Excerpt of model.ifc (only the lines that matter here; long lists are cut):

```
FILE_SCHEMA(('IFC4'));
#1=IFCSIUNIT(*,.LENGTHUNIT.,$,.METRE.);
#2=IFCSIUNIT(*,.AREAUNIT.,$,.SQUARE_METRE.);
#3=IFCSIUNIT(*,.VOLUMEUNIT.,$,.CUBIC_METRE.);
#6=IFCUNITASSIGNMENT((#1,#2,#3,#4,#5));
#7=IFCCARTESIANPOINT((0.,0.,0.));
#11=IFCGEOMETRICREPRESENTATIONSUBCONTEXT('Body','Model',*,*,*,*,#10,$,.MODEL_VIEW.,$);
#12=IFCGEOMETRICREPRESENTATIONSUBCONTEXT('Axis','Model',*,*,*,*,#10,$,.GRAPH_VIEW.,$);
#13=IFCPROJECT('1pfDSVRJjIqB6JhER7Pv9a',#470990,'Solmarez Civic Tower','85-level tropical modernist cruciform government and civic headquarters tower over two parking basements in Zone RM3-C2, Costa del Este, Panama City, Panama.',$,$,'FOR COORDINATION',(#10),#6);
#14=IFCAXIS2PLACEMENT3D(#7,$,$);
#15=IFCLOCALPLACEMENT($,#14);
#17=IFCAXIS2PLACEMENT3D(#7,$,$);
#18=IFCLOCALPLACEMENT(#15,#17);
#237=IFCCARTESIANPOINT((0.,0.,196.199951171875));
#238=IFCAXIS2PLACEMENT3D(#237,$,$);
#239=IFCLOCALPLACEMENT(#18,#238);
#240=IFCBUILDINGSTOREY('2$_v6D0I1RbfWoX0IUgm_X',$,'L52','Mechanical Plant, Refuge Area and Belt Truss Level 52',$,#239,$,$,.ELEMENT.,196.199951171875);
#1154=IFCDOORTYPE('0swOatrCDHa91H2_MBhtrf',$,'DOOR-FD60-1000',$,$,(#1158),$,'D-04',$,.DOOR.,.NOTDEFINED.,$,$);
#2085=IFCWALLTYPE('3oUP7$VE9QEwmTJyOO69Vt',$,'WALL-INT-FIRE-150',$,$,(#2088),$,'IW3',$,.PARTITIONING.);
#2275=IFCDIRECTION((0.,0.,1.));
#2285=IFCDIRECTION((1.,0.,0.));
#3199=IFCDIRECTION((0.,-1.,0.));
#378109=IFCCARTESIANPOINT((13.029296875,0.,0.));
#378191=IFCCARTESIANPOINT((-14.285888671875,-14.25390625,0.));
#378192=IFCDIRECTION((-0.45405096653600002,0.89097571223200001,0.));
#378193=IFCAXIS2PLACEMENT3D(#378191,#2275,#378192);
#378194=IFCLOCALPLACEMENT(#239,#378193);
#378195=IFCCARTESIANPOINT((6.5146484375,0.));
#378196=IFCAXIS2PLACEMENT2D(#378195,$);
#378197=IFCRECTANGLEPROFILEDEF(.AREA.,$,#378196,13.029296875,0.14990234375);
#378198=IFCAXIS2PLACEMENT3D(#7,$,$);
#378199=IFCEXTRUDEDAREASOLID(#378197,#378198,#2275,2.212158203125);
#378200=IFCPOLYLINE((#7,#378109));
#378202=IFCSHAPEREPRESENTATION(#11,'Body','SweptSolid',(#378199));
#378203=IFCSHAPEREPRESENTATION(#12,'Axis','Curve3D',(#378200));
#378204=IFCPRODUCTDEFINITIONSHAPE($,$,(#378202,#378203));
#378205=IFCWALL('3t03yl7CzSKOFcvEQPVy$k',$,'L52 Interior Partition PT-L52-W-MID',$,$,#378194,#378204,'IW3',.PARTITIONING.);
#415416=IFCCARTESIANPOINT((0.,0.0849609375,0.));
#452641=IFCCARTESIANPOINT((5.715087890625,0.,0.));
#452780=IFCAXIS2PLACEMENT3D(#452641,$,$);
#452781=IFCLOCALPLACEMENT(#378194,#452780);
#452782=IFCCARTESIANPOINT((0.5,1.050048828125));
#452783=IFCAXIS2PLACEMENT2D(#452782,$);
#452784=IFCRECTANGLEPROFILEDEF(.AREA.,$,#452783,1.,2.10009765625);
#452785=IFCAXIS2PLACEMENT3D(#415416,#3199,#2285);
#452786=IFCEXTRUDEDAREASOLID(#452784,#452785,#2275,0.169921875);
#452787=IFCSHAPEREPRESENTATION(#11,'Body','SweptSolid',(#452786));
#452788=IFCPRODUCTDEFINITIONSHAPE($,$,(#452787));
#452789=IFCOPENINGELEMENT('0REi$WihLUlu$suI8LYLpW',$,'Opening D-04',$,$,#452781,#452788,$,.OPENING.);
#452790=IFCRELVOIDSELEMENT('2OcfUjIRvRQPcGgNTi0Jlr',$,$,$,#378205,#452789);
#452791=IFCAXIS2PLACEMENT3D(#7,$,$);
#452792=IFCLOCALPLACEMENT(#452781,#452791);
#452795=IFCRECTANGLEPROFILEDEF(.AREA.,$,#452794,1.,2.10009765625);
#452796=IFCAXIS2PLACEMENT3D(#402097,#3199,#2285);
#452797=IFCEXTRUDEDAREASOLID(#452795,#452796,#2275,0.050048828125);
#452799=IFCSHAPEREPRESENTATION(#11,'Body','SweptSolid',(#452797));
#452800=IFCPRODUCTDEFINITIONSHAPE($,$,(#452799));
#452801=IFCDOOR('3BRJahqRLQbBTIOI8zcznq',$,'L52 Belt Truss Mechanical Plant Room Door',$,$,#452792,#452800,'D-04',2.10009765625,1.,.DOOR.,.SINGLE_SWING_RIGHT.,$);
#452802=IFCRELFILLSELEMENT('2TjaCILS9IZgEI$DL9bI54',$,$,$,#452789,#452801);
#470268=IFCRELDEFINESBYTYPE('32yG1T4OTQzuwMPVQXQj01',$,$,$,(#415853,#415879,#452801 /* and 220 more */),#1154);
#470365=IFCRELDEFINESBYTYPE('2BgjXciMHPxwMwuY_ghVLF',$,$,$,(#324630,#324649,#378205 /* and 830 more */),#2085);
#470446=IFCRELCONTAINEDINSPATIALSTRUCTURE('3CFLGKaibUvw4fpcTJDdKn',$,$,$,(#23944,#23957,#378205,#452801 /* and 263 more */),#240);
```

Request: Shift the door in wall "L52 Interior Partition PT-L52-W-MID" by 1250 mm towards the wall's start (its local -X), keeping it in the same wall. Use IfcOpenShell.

```python
import ifcopenshell
import ifcopenshell.api.geometry
import ifcopenshell.util.placement

model = ifcopenshell.open("model.ifc")

door = model.by_id(452801)
opening = door.FillsVoids[0].RelatingOpeningElement
wall = opening.VoidsElements[0].RelatingBuildingElement

wall_matrix = ifcopenshell.util.placement.get_local_placement(wall.ObjectPlacement)
shift = wall_matrix[:3, 0] * -1.25
before = ifcopenshell.util.placement.get_local_placement(door.ObjectPlacement)[:3, 3].copy()

# The door is placed relative to its opening, so it follows when the opening moves.
matrix = ifcopenshell.util.placement.get_local_placement(opening.ObjectPlacement)
matrix[:3, 3] += shift
ifcopenshell.api.geometry.edit_object_placement(
    model, product=opening, matrix=matrix, is_si=False, should_transform_children=True
)

after = ifcopenshell.util.placement.get_local_placement(door.ObjectPlacement)[:3, 3]
print("door moved by", (after - before).round(3) + 0.0)

model.write("model_v2.ifc")
```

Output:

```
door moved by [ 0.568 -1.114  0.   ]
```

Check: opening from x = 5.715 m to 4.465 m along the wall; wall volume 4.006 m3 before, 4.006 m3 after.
